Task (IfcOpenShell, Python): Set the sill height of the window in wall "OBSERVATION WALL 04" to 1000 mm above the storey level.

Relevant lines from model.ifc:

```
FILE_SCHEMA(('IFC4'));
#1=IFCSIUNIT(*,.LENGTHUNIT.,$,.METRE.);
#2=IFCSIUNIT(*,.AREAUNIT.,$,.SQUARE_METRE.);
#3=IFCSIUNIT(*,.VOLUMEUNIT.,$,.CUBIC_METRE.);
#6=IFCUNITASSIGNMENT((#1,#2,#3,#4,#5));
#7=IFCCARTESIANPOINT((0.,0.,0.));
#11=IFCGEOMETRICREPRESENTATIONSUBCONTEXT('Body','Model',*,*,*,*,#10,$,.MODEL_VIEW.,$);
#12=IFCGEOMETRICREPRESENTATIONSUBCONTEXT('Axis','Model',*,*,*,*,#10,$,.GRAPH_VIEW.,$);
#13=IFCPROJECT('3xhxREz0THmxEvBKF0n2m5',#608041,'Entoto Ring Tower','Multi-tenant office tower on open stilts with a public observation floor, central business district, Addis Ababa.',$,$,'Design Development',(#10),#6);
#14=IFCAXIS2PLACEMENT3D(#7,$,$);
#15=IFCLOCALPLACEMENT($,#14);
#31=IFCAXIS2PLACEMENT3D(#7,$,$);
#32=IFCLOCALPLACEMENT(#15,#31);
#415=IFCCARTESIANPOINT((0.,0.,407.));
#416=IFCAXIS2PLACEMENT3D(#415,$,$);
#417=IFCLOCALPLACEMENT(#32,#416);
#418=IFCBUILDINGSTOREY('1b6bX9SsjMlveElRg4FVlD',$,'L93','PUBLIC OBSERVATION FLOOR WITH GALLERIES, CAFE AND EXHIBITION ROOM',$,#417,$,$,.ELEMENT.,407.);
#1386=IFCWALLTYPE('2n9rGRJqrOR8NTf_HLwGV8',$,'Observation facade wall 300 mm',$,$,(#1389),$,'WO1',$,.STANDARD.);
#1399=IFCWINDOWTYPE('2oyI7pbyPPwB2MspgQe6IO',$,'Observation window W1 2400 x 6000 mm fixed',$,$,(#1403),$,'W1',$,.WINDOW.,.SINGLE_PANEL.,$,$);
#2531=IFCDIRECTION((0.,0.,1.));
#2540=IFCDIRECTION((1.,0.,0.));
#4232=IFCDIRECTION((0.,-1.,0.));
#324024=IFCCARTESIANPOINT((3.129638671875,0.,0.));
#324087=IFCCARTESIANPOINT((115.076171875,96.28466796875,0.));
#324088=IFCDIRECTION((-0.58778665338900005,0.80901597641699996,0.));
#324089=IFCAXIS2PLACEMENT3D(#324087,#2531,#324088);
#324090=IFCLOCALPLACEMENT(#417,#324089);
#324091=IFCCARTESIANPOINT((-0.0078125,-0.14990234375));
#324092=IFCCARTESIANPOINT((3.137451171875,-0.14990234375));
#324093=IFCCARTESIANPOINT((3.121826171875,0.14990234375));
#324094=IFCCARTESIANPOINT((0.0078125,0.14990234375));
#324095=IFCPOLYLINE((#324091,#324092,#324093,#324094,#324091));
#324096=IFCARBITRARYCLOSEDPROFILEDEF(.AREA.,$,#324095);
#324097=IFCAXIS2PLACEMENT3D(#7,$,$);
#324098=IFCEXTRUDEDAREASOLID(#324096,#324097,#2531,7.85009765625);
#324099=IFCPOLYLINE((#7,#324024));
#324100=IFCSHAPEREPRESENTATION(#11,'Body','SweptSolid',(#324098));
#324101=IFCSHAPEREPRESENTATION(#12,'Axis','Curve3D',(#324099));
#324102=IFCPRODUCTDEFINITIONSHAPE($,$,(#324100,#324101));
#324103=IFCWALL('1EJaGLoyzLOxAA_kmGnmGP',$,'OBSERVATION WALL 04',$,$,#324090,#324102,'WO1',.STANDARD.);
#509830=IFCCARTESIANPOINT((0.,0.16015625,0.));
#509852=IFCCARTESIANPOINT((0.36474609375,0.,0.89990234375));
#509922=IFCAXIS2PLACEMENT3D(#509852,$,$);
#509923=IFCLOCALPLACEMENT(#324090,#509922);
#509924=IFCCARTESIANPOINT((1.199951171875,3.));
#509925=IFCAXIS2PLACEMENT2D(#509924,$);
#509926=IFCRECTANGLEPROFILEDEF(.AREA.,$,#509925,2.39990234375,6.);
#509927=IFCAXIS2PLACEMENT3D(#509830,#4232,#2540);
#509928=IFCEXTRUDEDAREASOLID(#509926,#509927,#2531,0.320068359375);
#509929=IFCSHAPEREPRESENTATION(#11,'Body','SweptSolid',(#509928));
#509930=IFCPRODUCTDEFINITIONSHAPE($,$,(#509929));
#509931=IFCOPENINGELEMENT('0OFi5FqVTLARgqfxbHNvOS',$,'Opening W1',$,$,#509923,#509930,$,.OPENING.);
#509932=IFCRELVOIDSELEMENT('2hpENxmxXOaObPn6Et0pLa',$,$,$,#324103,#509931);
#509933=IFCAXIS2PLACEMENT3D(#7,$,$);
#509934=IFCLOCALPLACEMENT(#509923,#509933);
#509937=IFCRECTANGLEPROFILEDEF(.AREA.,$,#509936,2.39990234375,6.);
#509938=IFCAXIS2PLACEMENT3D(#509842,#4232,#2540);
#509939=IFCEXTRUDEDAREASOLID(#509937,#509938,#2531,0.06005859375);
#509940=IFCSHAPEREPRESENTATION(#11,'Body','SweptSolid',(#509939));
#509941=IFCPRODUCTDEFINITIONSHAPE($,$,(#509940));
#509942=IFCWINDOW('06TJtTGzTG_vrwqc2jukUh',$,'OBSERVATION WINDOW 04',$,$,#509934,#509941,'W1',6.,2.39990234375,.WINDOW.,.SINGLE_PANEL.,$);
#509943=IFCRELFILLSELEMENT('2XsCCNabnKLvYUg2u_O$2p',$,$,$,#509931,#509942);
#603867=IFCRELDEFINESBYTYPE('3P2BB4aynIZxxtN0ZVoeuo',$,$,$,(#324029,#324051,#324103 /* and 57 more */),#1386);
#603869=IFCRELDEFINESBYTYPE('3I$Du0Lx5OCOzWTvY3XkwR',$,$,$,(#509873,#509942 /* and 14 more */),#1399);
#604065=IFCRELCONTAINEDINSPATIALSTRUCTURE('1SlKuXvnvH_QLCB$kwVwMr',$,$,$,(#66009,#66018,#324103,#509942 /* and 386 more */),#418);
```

```python
import numpy as np
import ifcopenshell
import ifcopenshell.api.geometry
import ifcopenshell.geom
import ifcopenshell.util.element
import ifcopenshell.util.placement
import ifcopenshell.util.shape
import ifcopenshell.util.unit

model = ifcopenshell.open("model.ifc")
unit_scale = ifcopenshell.util.unit.calculate_unit_scale(model)

window = model.by_id(509942)
opening = window.FillsVoids[0].RelatingOpeningElement
storey = ifcopenshell.util.element.get_container(window, ifc_class="IfcBuildingStorey")
level = ifcopenshell.util.placement.get_local_placement(storey.ObjectPlacement)[2, 3]

# The opening's origin need not be at the sill, so measure its lowest point.
shape = ifcopenshell.geom.create_shape(ifcopenshell.geom.settings(), opening)
bottom = ifcopenshell.util.shape.get_shape_bottom_elevation(shape, shape.geometry) / unit_scale
dz = level + 1 / unit_scale - bottom

shift = np.array([0.0, 0.0, dz])
# The window is placed relative to its opening, so it follows when the opening moves.
matrix = ifcopenshell.util.placement.get_local_placement(opening.ObjectPlacement)
matrix[:3, 3] += shift
ifcopenshell.api.geometry.edit_object_placement(
    model, product=opening, matrix=matrix, is_si=False, should_transform_children=True
)

print(f"moved by {dz * unit_scale:+.3f} m")

model.write("model_v2.ifc")
```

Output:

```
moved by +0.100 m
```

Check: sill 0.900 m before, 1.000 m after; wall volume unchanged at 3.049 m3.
